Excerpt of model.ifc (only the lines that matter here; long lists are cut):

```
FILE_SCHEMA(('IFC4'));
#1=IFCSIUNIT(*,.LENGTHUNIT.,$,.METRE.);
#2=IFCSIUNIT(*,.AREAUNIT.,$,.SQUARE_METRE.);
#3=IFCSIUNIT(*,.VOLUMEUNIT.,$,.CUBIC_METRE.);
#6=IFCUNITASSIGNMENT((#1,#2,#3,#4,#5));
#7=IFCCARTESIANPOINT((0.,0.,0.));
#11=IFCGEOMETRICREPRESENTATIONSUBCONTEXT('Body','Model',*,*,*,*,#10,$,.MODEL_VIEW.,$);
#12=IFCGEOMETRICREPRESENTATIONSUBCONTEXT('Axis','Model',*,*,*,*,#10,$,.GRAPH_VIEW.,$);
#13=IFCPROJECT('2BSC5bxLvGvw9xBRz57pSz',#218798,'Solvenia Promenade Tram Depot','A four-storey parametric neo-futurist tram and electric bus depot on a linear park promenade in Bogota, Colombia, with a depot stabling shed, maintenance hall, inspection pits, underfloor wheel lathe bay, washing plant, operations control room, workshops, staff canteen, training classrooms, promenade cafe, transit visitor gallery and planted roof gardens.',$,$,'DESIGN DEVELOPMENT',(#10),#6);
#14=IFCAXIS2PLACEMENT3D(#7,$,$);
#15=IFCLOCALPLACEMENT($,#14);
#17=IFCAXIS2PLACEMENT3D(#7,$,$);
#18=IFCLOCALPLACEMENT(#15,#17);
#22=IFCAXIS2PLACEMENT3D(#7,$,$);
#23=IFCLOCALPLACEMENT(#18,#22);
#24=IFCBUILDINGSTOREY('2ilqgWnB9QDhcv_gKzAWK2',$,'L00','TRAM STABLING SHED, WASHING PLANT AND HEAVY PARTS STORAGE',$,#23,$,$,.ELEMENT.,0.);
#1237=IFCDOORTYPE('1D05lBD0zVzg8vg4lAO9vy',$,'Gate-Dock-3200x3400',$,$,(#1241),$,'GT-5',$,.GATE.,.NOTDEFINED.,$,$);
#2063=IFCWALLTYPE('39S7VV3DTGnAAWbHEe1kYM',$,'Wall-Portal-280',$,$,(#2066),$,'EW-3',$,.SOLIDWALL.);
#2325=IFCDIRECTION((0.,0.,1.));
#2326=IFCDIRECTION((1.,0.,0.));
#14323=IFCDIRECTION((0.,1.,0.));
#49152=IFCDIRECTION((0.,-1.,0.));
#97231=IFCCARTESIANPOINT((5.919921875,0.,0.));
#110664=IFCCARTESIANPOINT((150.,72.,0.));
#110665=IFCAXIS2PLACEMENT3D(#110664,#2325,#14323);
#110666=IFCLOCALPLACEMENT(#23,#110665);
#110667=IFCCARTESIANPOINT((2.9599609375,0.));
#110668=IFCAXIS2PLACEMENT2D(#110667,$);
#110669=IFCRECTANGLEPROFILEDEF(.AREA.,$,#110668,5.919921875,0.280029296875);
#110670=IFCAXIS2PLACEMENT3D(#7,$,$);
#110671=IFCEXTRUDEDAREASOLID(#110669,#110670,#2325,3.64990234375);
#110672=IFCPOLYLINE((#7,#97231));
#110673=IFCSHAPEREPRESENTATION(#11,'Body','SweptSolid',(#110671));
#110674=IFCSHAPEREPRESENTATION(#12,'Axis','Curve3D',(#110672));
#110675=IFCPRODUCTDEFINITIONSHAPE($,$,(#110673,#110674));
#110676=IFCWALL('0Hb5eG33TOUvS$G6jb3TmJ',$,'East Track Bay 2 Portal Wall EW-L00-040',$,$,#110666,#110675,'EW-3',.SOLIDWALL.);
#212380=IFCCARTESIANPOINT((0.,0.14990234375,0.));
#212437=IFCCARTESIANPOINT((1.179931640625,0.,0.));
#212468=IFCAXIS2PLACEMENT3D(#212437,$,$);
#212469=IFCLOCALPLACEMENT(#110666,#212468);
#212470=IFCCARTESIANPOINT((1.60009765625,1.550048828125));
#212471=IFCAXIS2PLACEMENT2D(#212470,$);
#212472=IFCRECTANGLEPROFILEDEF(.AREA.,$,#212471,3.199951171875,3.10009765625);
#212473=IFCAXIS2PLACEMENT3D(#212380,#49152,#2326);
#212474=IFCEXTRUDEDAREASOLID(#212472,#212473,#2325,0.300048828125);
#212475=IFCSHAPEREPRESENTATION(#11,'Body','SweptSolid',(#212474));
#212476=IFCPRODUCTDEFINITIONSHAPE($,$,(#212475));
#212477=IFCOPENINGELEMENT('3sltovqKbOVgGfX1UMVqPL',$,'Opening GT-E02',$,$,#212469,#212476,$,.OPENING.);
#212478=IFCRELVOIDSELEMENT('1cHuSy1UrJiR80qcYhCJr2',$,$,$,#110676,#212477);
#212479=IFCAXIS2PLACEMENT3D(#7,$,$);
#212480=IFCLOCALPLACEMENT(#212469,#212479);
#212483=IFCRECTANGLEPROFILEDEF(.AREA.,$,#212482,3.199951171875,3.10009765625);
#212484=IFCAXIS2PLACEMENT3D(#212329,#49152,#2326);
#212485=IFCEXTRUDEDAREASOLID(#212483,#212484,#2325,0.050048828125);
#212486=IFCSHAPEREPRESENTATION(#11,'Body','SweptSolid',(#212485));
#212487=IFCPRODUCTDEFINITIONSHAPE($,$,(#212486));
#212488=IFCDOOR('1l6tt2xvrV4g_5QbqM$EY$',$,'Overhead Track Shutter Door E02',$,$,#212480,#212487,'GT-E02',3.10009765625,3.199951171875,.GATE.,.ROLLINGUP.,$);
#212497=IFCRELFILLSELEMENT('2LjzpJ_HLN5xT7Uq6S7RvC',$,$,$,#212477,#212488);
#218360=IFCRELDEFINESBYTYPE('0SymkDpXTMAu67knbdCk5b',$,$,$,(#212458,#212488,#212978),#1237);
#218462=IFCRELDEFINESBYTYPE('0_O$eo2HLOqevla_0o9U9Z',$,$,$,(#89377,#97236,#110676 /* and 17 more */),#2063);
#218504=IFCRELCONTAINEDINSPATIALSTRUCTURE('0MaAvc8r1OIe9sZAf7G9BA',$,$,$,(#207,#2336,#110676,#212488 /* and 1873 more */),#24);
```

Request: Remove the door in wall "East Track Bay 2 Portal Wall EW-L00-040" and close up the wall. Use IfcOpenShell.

```python
import ifcopenshell
import ifcopenshell.api.feature
import ifcopenshell.api.root
import ifcopenshell.geom
import ifcopenshell.util.shape

model = ifcopenshell.open("model.ifc")
settings = ifcopenshell.geom.settings()


def volume(element):
    """Net volume in cubic metres, openings subtracted."""
    shape = ifcopenshell.geom.create_shape(settings, element)
    return ifcopenshell.util.shape.get_volume(shape.geometry)


door = model.by_guid("1l6tt2xvrV4g_5QbqM$EY$")
opening = door.FillsVoids[0].RelatingOpeningElement
wall = opening.VoidsElements[0].RelatingBuildingElement
before = volume(wall)

ifcopenshell.api.root.remove_product(model, product=door)
ifcopenshell.api.feature.remove_feature(model, feature=opening)

after = volume(wall)

print(f"wall volume {before:.3f} -> {after:.3f} m3")

model.write("model_edited.ifc")
```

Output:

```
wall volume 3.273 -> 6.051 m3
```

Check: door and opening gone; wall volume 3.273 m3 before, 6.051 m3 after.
